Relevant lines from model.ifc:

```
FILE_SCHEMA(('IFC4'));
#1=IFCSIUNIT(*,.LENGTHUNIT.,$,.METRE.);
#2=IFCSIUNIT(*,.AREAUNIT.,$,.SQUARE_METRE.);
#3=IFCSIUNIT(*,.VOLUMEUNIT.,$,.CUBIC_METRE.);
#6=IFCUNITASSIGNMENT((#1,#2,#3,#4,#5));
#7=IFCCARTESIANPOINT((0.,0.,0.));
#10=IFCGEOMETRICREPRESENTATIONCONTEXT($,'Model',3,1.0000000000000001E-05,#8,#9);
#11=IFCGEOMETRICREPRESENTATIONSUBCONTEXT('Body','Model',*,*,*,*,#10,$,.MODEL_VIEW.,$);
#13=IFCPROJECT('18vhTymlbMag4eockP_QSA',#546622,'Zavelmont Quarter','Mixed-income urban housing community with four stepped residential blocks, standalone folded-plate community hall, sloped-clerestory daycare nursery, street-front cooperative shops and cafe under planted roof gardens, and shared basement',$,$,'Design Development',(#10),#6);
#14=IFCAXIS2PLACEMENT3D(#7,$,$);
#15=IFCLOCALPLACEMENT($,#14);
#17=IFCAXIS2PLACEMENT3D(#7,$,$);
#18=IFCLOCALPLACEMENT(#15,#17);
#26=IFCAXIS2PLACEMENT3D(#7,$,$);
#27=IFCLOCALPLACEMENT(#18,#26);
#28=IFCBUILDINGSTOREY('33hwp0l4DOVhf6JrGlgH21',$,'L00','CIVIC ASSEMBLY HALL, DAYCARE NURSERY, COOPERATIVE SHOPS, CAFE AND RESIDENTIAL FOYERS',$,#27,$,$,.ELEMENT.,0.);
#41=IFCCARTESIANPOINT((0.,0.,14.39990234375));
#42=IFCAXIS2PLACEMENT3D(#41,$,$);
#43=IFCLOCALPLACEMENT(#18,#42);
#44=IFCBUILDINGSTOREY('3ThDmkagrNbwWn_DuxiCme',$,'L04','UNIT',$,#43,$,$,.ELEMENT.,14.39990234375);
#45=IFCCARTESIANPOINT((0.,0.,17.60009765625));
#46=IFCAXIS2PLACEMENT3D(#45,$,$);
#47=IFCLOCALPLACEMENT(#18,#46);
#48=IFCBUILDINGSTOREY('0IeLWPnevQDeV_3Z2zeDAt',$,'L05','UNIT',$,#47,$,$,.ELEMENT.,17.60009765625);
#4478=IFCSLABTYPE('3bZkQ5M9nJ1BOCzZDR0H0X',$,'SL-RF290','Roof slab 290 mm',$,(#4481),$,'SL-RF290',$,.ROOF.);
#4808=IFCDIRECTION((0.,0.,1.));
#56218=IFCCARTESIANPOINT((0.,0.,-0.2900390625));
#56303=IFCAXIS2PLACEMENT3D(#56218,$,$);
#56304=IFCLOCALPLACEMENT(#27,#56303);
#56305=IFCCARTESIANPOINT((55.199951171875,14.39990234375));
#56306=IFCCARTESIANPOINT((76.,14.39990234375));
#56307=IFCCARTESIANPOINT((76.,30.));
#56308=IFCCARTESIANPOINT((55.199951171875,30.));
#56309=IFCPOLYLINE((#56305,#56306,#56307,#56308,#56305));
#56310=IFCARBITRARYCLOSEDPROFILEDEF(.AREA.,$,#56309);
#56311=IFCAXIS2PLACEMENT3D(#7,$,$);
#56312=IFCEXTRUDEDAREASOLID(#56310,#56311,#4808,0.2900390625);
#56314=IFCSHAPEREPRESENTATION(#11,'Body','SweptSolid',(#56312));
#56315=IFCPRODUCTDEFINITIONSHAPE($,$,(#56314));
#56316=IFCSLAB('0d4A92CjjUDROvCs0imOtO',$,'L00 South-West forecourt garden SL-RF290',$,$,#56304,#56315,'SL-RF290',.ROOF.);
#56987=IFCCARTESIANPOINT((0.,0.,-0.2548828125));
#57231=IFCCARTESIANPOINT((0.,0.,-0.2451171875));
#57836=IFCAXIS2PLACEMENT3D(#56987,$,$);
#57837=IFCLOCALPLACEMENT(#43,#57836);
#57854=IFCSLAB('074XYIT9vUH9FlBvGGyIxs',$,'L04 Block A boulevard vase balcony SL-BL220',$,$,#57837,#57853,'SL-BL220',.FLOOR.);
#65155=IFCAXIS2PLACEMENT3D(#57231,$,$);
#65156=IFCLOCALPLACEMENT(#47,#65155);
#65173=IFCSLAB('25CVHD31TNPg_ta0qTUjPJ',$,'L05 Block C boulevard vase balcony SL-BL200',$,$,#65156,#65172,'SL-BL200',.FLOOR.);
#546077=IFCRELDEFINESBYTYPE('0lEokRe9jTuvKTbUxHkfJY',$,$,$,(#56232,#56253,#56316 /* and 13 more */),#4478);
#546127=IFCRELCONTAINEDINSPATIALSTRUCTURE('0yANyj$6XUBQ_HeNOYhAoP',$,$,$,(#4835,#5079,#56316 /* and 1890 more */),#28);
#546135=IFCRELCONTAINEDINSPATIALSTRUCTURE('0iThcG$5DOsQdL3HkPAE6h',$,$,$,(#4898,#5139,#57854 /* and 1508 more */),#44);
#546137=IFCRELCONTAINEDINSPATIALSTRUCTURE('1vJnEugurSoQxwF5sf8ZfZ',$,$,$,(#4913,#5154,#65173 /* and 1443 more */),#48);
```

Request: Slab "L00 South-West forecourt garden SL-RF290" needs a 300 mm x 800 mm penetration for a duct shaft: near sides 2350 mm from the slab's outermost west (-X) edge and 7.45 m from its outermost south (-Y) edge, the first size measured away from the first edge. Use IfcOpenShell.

```python
import numpy as np
import ifcopenshell
import ifcopenshell.api.feature
import ifcopenshell.api.geometry
import ifcopenshell.api.root
import ifcopenshell.geom
import ifcopenshell.util.placement
import ifcopenshell.util.representation
import ifcopenshell.util.shape
import ifcopenshell.util.unit

model = ifcopenshell.open("model.ifc")
unit_scale = ifcopenshell.util.unit.calculate_unit_scale(model)
settings = ifcopenshell.geom.settings()


def volume(element):
    """Net volume in cubic metres, openings subtracted."""
    shape = ifcopenshell.geom.create_shape(settings, element)
    return ifcopenshell.util.shape.get_volume(shape.geometry)


slab = model.by_guid("0d4A92CjjUDROvCs0imOtO")
before = volume(slab)

# Extent in the slab's own axes, in metres. The edges named are its -X and -Y sides.
slab_shape = ifcopenshell.geom.create_shape(settings, slab)
vertices = ifcopenshell.util.shape.get_vertices(slab_shape.geometry)
x_min, y_min, bottom = vertices.min(axis=0)
top = vertices[:, 2].max()

opening = ifcopenshell.api.root.create_entity(model, ifc_class="IfcOpeningElement", name="Duct shaft opening", predefined_type="OPENING")
context = ifcopenshell.util.representation.get_context(model, "Model", "Body", "MODEL_VIEW")
width, depth = 0.3, 0.8
outline = [(0.0, 0.0), (width, 0.0), (width, depth), (0.0, depth), (0.0, 0.0)]
# Overshoot both faces by 50 mm so the cut is clean.
shape = ifcopenshell.api.geometry.add_slab_representation(
    model, context=context, depth=top - bottom + 0.1, polyline=outline
)
ifcopenshell.api.geometry.assign_representation(model, product=opening, representation=shape)

matrix = ifcopenshell.util.placement.get_local_placement(slab.ObjectPlacement)
matrix[:, 3] = matrix @ np.append(np.array([x_min + 2.35, y_min + 7.45, bottom - 0.05]) / unit_scale, 1.0)
ifcopenshell.api.geometry.edit_object_placement(model, product=opening, matrix=matrix, is_si=False)
ifcopenshell.api.feature.add_feature(model, feature=opening, element=slab)

after = volume(slab)

print(f"slab volume {before:.3f} -> {after:.3f} m3")

model.write("model_edited.ifc")
```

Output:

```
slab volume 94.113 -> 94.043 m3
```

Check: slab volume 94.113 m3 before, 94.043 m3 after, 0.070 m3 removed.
